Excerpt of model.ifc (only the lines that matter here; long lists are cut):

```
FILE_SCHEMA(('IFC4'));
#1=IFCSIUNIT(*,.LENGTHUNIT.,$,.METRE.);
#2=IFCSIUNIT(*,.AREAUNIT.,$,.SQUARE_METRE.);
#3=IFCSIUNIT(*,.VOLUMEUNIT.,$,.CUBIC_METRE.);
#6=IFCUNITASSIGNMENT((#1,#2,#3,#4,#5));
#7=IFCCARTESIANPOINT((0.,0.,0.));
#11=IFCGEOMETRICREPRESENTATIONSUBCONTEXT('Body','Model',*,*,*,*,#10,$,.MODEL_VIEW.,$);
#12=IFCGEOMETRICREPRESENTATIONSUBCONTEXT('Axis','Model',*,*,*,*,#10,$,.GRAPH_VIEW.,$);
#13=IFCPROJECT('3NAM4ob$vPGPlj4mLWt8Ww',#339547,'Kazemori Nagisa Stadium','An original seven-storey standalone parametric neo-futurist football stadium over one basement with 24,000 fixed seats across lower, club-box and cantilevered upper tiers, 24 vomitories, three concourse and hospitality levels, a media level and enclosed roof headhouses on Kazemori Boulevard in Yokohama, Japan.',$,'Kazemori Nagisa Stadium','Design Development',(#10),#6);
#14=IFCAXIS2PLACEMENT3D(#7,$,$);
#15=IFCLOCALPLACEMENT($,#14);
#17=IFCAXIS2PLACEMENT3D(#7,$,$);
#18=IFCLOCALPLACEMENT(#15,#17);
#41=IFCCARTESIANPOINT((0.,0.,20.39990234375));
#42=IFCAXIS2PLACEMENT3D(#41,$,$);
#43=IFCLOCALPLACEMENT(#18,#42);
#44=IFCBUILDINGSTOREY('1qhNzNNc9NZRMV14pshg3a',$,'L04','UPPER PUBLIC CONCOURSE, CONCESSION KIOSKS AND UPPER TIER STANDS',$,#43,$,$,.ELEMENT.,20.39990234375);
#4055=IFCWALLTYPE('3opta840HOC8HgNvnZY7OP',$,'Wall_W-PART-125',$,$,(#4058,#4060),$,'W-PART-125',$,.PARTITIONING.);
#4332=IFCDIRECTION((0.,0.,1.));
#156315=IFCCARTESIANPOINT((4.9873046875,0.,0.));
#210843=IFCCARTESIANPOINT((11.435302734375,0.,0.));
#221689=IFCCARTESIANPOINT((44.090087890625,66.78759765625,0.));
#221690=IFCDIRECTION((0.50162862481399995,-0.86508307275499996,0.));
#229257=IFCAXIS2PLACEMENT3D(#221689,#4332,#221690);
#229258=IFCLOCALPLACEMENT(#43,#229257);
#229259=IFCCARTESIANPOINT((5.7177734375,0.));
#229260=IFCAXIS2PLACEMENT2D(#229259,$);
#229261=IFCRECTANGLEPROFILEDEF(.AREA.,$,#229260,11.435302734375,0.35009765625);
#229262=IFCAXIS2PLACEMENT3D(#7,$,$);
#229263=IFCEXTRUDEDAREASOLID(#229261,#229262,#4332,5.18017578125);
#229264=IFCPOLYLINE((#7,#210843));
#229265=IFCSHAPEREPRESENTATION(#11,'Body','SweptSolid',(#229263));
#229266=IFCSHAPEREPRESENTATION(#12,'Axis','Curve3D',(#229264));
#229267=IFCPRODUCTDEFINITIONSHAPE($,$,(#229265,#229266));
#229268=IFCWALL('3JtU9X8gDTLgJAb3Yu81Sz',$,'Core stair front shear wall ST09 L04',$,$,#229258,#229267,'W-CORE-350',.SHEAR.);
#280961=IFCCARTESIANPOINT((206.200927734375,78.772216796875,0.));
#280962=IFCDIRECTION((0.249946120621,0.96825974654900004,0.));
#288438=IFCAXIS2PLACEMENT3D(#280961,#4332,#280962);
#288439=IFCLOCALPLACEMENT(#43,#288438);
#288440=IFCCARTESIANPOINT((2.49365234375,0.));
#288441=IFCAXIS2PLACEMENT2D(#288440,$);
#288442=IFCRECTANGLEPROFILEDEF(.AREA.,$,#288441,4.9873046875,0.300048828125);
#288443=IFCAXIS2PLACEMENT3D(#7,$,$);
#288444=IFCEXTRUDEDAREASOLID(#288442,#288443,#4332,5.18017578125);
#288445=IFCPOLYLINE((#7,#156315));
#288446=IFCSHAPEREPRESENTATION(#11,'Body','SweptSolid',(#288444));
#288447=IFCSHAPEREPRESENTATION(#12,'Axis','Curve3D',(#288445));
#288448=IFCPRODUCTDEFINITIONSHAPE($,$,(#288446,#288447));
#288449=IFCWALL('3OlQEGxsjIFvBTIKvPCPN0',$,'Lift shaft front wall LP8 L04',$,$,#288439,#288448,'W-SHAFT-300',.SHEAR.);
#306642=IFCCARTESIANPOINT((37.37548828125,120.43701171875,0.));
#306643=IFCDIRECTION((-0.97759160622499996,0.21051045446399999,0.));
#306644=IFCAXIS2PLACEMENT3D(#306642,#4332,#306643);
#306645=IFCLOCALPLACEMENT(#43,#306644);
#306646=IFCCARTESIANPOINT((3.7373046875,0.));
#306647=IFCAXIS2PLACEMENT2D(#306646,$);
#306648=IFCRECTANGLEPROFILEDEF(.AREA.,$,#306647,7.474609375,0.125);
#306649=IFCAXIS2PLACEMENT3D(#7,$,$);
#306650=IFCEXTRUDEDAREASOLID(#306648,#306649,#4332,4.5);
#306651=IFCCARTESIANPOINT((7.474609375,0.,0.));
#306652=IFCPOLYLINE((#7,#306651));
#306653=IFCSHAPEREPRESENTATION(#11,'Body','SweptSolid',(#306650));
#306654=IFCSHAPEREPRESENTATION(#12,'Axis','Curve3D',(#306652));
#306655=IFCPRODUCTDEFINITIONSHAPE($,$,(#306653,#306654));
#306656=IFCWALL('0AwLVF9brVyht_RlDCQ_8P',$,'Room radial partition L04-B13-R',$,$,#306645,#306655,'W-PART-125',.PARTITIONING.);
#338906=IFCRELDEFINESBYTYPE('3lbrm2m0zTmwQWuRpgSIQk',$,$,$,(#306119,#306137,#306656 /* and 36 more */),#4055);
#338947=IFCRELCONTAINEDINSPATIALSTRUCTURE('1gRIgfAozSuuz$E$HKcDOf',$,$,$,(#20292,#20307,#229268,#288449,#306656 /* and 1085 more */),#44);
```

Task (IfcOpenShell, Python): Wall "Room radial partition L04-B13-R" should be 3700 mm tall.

```python
import ifcopenshell
import ifcopenshell.geom
import ifcopenshell.util.representation
import ifcopenshell.util.shape
import ifcopenshell.util.unit

model = ifcopenshell.open("model.ifc")
unit_scale = ifcopenshell.util.unit.calculate_unit_scale(model)
settings = ifcopenshell.geom.settings()


def volume(element):
    """Net volume in cubic metres, openings subtracted."""
    shape = ifcopenshell.geom.create_shape(settings, element)
    return ifcopenshell.util.shape.get_volume(shape.geometry)


wall = model.by_guid("0AwLVF9brVyht_RlDCQ_8P")
before = volume(wall)

body = ifcopenshell.util.representation.get_representation(wall, "Model", "Body")
solid = body.Items[0]
old_height = solid.Depth
solid.Depth = 3.7 / unit_scale
after = volume(wall)

print(f"height {old_height:g} -> {solid.Depth:g}, volume {before:.3f} -> {after:.3f} m3")

model.write("model_rev.ifc")
```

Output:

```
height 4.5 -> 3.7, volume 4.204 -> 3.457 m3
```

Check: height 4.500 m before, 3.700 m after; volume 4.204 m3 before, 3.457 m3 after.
